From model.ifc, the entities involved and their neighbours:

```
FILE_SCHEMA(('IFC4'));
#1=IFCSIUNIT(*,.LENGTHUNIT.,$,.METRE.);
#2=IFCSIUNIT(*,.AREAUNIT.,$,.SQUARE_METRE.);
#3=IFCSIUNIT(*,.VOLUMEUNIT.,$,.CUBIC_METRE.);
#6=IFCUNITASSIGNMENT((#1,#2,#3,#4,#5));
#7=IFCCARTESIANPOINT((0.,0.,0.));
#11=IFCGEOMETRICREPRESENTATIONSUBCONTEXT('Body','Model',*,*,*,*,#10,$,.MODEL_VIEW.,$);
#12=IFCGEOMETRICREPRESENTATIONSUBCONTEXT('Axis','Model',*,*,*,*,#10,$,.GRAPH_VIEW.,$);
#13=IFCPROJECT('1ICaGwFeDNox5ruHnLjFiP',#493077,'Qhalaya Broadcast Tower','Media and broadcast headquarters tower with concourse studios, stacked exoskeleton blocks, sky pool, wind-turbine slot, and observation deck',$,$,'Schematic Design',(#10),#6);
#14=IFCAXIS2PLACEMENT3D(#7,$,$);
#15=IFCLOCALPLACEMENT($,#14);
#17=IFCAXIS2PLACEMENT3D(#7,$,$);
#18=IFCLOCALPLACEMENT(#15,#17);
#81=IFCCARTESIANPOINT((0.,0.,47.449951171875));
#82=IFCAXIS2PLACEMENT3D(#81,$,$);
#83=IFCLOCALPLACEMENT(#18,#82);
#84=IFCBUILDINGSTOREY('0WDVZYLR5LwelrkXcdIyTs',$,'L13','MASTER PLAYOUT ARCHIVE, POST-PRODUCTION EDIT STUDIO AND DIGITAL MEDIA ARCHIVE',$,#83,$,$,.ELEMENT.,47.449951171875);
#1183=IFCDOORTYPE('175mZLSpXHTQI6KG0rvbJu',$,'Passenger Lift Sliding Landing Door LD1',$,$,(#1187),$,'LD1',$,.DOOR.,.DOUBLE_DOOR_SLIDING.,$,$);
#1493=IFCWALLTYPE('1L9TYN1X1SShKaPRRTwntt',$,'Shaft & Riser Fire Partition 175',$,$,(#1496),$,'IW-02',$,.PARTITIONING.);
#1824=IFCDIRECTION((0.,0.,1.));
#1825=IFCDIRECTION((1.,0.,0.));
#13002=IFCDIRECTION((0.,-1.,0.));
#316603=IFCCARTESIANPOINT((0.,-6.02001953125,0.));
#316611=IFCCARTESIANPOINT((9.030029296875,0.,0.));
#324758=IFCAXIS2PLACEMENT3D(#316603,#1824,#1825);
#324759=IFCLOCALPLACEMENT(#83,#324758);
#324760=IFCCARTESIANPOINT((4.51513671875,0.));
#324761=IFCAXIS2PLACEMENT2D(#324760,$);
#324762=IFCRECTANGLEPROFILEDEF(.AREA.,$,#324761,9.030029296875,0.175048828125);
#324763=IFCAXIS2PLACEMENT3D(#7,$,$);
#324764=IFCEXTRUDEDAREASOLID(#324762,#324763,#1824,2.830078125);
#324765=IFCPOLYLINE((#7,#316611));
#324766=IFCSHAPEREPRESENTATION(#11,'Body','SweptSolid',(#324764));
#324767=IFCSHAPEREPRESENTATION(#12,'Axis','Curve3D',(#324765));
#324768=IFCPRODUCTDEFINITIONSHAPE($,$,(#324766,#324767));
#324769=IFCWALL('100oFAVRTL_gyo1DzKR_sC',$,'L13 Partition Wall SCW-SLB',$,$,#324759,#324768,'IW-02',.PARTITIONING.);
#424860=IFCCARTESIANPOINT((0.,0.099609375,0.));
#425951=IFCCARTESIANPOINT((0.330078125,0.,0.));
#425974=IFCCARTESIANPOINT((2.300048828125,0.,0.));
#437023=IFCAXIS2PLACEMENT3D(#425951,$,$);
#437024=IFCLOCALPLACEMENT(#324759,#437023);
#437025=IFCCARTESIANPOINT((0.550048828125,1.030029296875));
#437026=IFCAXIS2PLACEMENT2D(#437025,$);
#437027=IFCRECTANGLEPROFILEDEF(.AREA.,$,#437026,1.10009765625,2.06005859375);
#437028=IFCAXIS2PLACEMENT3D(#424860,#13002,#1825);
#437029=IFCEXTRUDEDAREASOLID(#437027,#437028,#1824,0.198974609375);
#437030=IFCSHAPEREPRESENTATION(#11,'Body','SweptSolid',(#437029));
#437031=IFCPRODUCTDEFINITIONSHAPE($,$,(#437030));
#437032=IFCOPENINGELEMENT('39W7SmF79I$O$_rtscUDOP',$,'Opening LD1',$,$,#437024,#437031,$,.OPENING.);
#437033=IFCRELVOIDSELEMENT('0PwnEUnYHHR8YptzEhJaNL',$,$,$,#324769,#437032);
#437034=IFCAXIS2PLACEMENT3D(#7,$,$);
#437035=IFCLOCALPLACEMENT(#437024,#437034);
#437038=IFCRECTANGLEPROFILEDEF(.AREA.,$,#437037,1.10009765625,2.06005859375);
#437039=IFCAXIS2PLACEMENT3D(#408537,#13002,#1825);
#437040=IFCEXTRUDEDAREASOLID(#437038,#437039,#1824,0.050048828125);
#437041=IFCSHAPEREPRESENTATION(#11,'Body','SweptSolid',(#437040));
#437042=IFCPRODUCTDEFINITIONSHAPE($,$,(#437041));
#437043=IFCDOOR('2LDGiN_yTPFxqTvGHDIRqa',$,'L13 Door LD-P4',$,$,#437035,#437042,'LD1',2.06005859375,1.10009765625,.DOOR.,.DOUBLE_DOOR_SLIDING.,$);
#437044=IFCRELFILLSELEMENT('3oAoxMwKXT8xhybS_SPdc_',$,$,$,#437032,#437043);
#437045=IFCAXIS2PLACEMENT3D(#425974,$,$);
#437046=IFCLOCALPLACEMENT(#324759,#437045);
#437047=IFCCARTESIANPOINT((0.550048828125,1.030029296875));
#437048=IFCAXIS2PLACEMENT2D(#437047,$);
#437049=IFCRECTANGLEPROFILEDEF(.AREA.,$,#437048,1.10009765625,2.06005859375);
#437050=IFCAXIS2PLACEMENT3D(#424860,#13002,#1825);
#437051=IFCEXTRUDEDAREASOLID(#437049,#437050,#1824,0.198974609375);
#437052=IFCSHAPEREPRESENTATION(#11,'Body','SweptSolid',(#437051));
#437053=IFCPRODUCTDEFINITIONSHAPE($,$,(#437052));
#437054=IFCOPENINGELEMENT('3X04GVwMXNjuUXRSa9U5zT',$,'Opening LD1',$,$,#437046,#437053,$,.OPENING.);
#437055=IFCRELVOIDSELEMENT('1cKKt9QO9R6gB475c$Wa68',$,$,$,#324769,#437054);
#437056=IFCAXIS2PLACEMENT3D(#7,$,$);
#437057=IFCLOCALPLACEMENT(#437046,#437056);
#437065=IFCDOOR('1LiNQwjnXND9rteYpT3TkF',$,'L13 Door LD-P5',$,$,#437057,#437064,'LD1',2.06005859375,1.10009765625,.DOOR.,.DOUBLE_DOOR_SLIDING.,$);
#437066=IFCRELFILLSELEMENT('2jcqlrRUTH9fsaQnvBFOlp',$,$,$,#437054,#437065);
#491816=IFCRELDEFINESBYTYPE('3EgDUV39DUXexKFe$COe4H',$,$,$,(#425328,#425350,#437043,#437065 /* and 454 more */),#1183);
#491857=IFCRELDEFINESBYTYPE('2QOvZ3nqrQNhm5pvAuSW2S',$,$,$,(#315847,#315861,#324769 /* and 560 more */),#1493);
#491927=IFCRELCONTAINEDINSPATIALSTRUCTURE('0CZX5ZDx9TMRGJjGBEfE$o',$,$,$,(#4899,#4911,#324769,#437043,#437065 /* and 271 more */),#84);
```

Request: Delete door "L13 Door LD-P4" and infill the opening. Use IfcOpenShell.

```python
import ifcopenshell
import ifcopenshell.api.feature
import ifcopenshell.api.root
import ifcopenshell.geom
import ifcopenshell.util.shape

model = ifcopenshell.open("model.ifc")
settings = ifcopenshell.geom.settings()


def volume(element):
    """Net volume in cubic metres, openings subtracted."""
    shape = ifcopenshell.geom.create_shape(settings, element)
    return ifcopenshell.util.shape.get_volume(shape.geometry)


door = model.by_guid("2LDGiN_yTPFxqTvGHDIRqa")
opening = door.FillsVoids[0].RelatingOpeningElement
wall = opening.VoidsElements[0].RelatingBuildingElement
before = volume(wall)

ifcopenshell.api.root.remove_product(model, product=door)
ifcopenshell.api.feature.remove_feature(model, feature=opening)

after = volume(wall)

print(f"wall volume {before:.3f} -> {after:.3f} m3")

model.write("model-out.ifc")
```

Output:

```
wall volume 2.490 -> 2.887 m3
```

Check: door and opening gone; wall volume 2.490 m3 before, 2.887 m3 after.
